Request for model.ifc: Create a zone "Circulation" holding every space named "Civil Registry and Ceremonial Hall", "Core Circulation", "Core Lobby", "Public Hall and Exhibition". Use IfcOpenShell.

First a look at what the model holds.

```python
import ifcopenshell

model = ifcopenshell.open("model.ifc")
print(model.schema)
seen = {}
for space in model.by_type("IfcSpace"):
    seen[space.LongName] = seen.get(space.LongName, 0) + 1
for name, count in sorted(seen.items(), key=str):
    print(count, "x", name)
print("zones:", [z.Name for z in model.by_type("IfcZone")][:20])
```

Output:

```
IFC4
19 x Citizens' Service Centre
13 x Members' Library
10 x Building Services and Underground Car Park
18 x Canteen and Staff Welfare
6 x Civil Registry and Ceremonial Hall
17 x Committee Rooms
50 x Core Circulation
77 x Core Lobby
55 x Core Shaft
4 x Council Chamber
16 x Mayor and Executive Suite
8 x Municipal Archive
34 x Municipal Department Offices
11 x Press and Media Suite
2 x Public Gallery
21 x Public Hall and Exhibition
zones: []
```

```python
import ifcopenshell
import ifcopenshell.api.group
import ifcopenshell.api.root

model = ifcopenshell.open("model.ifc")

names = {"Civil Registry and Ceremonial Hall", "Core Circulation", "Core Lobby", "Public Hall and Exhibition"}
spaces = [s for s in model.by_type("IfcSpace") if s.LongName in names]

zone = ifcopenshell.api.root.create_entity(model, ifc_class="IfcZone", name="Circulation")
ifcopenshell.api.group.assign_group(model, products=spaces, group=zone)
print(len(spaces), "spaces in", zone.Name)

model.write("model_edited.ifc")
```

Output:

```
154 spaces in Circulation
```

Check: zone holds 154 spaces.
